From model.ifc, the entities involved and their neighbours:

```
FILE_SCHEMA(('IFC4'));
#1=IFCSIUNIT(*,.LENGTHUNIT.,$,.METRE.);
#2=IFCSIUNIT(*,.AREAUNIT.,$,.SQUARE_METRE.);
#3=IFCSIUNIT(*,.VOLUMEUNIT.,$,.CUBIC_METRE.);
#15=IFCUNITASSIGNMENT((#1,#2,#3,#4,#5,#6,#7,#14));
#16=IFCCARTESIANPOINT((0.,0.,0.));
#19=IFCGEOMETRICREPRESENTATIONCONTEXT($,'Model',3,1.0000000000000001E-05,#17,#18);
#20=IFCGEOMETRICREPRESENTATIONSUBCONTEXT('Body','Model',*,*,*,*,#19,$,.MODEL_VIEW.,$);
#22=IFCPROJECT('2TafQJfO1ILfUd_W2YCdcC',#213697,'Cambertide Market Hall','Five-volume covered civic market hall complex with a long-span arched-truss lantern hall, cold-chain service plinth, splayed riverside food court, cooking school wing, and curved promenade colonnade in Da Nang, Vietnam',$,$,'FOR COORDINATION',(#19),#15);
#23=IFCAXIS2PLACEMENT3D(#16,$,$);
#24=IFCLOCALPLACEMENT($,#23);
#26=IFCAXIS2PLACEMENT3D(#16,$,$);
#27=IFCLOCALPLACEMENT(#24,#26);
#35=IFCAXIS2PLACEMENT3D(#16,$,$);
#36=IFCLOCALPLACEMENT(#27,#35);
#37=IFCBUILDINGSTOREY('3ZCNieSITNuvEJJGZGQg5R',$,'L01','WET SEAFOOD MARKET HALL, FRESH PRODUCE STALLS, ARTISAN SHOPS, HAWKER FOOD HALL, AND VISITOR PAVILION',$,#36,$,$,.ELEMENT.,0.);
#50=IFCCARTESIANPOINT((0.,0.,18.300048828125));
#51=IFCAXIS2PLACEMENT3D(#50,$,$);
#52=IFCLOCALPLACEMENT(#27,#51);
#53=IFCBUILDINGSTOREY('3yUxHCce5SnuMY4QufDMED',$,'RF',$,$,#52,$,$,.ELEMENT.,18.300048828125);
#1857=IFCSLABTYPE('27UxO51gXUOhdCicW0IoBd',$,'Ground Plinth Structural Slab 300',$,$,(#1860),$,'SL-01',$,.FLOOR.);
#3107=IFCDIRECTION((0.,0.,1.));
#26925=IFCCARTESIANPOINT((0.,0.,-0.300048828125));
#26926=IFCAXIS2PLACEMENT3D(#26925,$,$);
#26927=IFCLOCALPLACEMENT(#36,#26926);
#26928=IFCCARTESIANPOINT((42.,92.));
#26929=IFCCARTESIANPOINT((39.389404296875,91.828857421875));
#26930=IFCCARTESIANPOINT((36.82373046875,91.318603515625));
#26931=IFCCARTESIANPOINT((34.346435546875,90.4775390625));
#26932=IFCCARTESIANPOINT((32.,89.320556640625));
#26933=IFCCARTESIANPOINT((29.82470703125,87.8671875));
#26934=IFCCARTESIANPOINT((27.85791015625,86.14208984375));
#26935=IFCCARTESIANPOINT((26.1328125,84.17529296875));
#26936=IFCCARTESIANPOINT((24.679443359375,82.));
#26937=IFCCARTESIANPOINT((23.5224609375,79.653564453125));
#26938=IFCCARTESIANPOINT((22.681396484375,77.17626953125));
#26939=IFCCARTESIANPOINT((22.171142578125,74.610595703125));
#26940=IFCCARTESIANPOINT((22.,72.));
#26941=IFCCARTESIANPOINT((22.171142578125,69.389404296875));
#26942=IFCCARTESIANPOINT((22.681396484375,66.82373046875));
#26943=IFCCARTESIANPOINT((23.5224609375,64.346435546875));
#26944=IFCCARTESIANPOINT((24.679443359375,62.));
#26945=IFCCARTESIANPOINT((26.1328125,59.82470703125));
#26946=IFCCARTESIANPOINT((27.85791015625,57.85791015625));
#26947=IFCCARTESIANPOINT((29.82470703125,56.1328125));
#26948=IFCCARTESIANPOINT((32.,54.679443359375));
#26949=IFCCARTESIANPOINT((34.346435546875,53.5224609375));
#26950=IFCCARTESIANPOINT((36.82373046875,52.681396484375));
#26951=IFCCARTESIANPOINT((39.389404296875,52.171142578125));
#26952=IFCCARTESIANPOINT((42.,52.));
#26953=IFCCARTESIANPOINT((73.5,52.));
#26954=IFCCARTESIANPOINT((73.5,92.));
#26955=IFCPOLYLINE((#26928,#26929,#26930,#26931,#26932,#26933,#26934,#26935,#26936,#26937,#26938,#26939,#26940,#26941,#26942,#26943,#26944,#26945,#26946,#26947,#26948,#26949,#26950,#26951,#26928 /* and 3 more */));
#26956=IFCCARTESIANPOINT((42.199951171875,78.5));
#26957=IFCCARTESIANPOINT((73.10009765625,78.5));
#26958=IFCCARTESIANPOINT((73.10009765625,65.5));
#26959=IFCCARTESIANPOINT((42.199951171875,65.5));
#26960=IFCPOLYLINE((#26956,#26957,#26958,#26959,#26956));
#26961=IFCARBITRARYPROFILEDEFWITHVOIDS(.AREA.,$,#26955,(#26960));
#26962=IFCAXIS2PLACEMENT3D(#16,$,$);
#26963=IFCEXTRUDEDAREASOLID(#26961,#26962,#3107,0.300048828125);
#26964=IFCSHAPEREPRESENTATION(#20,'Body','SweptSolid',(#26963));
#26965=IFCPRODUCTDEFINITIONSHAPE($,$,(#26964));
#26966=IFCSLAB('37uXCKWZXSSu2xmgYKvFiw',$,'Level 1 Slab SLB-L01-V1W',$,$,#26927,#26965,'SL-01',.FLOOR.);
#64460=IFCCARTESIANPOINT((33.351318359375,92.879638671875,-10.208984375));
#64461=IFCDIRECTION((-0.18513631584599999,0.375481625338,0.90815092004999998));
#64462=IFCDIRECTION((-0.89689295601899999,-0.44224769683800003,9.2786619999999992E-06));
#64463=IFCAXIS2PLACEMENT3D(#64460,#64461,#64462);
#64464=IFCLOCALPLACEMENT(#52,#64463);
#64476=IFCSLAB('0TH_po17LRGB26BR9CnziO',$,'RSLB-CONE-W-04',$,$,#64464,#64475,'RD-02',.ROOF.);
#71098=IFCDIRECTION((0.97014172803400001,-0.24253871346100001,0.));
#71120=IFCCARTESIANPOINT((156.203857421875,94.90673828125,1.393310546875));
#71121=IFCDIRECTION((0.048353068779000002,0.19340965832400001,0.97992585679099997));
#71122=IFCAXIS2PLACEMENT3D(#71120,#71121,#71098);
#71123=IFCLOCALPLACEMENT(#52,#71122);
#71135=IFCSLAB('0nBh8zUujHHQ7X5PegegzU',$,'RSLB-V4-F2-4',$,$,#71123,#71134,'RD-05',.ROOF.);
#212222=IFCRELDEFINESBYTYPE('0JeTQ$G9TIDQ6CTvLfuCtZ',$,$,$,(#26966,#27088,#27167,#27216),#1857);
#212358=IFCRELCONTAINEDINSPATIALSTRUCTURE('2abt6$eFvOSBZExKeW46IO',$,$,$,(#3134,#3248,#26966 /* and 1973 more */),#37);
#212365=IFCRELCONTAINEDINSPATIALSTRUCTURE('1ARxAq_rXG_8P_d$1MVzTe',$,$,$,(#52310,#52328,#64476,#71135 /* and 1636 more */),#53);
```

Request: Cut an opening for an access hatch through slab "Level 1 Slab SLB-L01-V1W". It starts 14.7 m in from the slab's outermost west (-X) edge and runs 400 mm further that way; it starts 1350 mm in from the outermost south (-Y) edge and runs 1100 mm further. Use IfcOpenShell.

```python
import numpy as np
import ifcopenshell
import ifcopenshell.api.feature
import ifcopenshell.api.geometry
import ifcopenshell.api.root
import ifcopenshell.geom
import ifcopenshell.util.placement
import ifcopenshell.util.representation
import ifcopenshell.util.shape
import ifcopenshell.util.unit

model = ifcopenshell.open("model.ifc")
unit_scale = ifcopenshell.util.unit.calculate_unit_scale(model)
settings = ifcopenshell.geom.settings()


def volume(element):
    """Net volume in cubic metres, openings subtracted."""
    shape = ifcopenshell.geom.create_shape(settings, element)
    return ifcopenshell.util.shape.get_volume(shape.geometry)


slab = model.by_guid("37uXCKWZXSSu2xmgYKvFiw")
before = volume(slab)

# Extent in the slab's own axes, in metres. The edges named are its -X and -Y sides.
slab_shape = ifcopenshell.geom.create_shape(settings, slab)
vertices = ifcopenshell.util.shape.get_vertices(slab_shape.geometry)
x_min, y_min, bottom = vertices.min(axis=0)
top = vertices[:, 2].max()

opening = ifcopenshell.api.root.create_entity(model, ifc_class="IfcOpeningElement", name="Access hatch opening", predefined_type="OPENING")
context = ifcopenshell.util.representation.get_context(model, "Model", "Body", "MODEL_VIEW")
width, depth = 0.4, 1.1
outline = [(0.0, 0.0), (width, 0.0), (width, depth), (0.0, depth), (0.0, 0.0)]
# Overshoot both faces by 50 mm so the cut is clean.
shape = ifcopenshell.api.geometry.add_slab_representation(
    model, context=context, depth=top - bottom + 0.1, polyline=outline
)
ifcopenshell.api.geometry.assign_representation(model, product=opening, representation=shape)

matrix = ifcopenshell.util.placement.get_local_placement(slab.ObjectPlacement)
matrix[:, 3] = matrix @ np.append(np.array([x_min + 14.7, y_min + 1.35, bottom - 0.05]) / unit_scale, 1.0)
ifcopenshell.api.geometry.edit_object_placement(model, product=opening, matrix=matrix, is_si=False)
ifcopenshell.api.feature.add_feature(model, feature=opening, element=slab)

after = volume(slab)

print(f"slab volume {before:.3f} -> {after:.3f} m3")

model.write("model_edited.ifc")
```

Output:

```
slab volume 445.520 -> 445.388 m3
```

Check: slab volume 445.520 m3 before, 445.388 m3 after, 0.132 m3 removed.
